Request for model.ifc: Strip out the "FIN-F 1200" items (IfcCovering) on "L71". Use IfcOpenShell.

First a look at what the model holds.

```python
import ifcopenshell
import ifcopenshell.util.element

model = ifcopenshell.open("model.ifc")
print(model.schema)
storey = next(s for s in model.by_type("IfcBuildingStorey") if s.Name == "L71")
coverings = [e for e in ifcopenshell.util.element.get_decomposition(storey) if e.is_a("IfcCovering")]
seen = {}
for e in coverings:
    element_type = ifcopenshell.util.element.get_type(e)
    name = element_type.Name if element_type not in (None, e) else None
    seen[name] = seen.get(name, 0) + 1
for name, count in sorted(seen.items(), key=str):
    print(count, "x", name)
```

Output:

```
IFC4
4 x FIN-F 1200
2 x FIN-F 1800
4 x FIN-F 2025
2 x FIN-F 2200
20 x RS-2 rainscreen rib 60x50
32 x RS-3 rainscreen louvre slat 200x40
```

```python
import ifcopenshell
import ifcopenshell.api.root
import ifcopenshell.util.element

model = ifcopenshell.open("model.ifc")

storey = next(s for s in model.by_type("IfcBuildingStorey") if s.Name == "L71")
coverings = [e for e in ifcopenshell.util.element.get_decomposition(storey) if e.is_a("IfcCovering")]
targets = [e for e in coverings if (t := ifcopenshell.util.element.get_type(e)) not in (None, e) and t.Name == "FIN-F 1200"]

for e in targets:
    ifcopenshell.api.root.remove_product(model, product=e)
print(len(targets), "removed")

model.write("model_updated.ifc")
```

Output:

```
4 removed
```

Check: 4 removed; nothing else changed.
